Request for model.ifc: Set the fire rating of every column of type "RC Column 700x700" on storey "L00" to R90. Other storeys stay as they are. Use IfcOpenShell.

First a look at what the model holds.

```python
import ifcopenshell
import ifcopenshell.util.element

model = ifcopenshell.open("model.ifc")
print(model.schema)
storey = next(s for s in model.by_type("IfcBuildingStorey") if s.Name == "L00")
columns = [e for e in ifcopenshell.util.element.get_decomposition(storey) if e.is_a("IfcColumn")]
seen = {}
for e in columns:
    element_type = ifcopenshell.util.element.get_type(e)
    key = (element_type.Name if element_type != e and element_type else None, ifcopenshell.util.element.get_pset(e, "Pset_ColumnCommon", "FireRating"))
    seen[key] = seen.get(key, 0) + 1
for (name, value), count in sorted(seen.items(), key=str):
    print(count, "x", name, "|", value)
```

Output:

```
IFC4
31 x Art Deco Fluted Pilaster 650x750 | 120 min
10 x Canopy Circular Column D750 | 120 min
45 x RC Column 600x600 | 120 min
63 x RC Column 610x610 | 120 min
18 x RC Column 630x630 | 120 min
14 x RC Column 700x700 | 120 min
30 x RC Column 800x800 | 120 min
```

```python
import ifcopenshell
import ifcopenshell.api.pset
import ifcopenshell.util.element

model = ifcopenshell.open("model.ifc")

storey = next(s for s in model.by_type("IfcBuildingStorey") if s.Name == "L00")
columns = [e for e in ifcopenshell.util.element.get_decomposition(storey) if e.is_a("IfcColumn")]

count = 0
for e in columns:
    element_type = ifcopenshell.util.element.get_type(e)
    if element_type in (None, e) or element_type.Name != "RC Column 700x700":
        continue
    # add_pset returns the element's existing set when there is one.
    pset = ifcopenshell.api.pset.add_pset(model, product=e, name="Pset_ColumnCommon")
    ifcopenshell.api.pset.edit_pset(model, pset=pset, properties={"FireRating": "R90"})
    count += 1

print(count, "columns updated")

model.write("model_v2.ifc")
```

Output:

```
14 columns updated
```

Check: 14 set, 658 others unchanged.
